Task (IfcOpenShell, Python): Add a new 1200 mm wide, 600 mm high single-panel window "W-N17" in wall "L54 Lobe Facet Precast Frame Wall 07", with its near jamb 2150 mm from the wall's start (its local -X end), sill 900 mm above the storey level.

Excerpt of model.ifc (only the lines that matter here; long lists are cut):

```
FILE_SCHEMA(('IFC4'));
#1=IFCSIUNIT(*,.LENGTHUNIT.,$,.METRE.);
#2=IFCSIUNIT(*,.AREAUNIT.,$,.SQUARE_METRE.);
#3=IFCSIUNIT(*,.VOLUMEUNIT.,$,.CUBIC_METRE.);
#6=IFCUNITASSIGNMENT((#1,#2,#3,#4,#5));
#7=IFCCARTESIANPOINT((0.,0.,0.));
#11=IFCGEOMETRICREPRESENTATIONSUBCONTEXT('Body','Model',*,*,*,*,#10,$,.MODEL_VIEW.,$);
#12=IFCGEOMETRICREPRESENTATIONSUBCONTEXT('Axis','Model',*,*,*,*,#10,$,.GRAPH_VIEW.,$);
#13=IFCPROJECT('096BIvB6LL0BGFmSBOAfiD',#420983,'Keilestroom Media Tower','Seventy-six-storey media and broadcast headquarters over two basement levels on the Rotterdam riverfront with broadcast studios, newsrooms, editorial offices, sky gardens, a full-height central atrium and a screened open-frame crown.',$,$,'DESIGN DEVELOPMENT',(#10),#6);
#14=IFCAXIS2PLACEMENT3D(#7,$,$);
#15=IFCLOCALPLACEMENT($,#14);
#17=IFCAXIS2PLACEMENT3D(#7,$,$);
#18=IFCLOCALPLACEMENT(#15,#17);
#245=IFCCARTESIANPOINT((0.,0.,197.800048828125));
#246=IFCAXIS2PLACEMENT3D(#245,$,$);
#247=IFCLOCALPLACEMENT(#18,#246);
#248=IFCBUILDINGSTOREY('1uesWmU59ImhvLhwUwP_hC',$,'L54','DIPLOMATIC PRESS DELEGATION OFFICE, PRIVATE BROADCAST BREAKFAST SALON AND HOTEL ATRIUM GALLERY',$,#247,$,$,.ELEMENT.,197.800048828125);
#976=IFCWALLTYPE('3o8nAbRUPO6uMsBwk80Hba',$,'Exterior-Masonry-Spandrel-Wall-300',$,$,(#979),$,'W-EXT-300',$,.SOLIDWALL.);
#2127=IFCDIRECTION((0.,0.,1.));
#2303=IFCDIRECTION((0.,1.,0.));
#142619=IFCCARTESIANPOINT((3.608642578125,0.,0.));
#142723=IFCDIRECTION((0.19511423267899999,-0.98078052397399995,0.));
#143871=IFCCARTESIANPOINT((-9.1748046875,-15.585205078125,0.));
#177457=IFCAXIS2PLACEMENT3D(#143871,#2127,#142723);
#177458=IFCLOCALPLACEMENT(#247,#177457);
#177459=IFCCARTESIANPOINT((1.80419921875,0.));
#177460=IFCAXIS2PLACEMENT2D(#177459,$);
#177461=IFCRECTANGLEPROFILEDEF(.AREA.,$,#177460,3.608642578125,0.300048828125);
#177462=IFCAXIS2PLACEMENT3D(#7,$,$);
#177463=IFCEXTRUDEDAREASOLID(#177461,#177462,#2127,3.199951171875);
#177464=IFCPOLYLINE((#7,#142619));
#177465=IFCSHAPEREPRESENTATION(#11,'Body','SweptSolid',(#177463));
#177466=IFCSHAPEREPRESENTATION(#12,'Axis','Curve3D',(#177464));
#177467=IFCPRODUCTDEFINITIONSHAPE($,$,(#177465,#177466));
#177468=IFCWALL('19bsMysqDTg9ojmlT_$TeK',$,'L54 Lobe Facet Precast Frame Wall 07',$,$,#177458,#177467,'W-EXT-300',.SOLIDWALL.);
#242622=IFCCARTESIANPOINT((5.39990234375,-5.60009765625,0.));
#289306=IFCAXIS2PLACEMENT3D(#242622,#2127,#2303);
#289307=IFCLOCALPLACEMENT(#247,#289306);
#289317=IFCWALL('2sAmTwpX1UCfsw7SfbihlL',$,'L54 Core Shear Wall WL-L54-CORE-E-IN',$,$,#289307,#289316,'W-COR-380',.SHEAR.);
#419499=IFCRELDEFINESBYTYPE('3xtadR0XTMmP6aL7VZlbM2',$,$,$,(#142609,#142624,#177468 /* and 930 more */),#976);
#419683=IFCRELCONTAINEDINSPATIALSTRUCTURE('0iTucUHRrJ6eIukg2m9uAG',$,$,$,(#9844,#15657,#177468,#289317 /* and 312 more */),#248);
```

```python
import numpy as np
import ifcopenshell
import ifcopenshell.api.feature
import ifcopenshell.api.geometry
import ifcopenshell.api.root
import ifcopenshell.api.spatial
import ifcopenshell.geom
import ifcopenshell.util.element
import ifcopenshell.util.placement
import ifcopenshell.util.representation
import ifcopenshell.util.shape
import ifcopenshell.util.unit

model = ifcopenshell.open("model.ifc")
unit_scale = ifcopenshell.util.unit.calculate_unit_scale(model)
settings = ifcopenshell.geom.settings()


def volume(element):
    """Net volume in cubic metres, openings subtracted."""
    shape = ifcopenshell.geom.create_shape(settings, element)
    return ifcopenshell.util.shape.get_volume(shape.geometry)


wall = model.by_guid("19bsMysqDTg9ojmlT_$TeK")
storey = ifcopenshell.util.element.get_container(wall, ifc_class="IfcBuildingStorey")
context = ifcopenshell.util.representation.get_context(model, "Model", "Body", "MODEL_VIEW")
before = volume(wall)

width, height, from_end, sill = 1.2, 0.6, 2.15, 0.9  # metres

# The wall runs along its own X axis, and the end named is its -X end.
wall_shape = ifcopenshell.geom.create_shape(settings, wall)
x, y, z = ifcopenshell.util.shape.get_vertices(wall_shape.geometry).T
start = x.min() + from_end
face, thickness = float(y.min()), float(y.max() - y.min())
wall_matrix = ifcopenshell.util.placement.get_local_placement(wall.ObjectPlacement)
level = ifcopenshell.util.placement.get_local_placement(storey.ObjectPlacement)[2, 3]


def in_wall(x, y):
    """Placement at x, y metres in the wall's axes, at sill height."""
    matrix = wall_matrix.copy()
    matrix[:, 3] = wall_matrix @ np.array([x / unit_scale, y / unit_scale, 0.0, 1.0])
    matrix[2, 3] = level + sill / unit_scale
    return matrix


# Opening: a box that overshoots both wall faces by 50 mm.
opening = ifcopenshell.api.root.create_entity(model, ifc_class="IfcOpeningElement", predefined_type="OPENING")
box = ifcopenshell.api.geometry.add_wall_representation(
    model, context=context, length=width, height=height, thickness=thickness + 0.1
)
ifcopenshell.api.geometry.assign_representation(model, product=opening, representation=box)
ifcopenshell.api.geometry.edit_object_placement(model, product=opening, matrix=in_wall(start, face - 0.05), is_si=False)
ifcopenshell.api.feature.add_feature(model, feature=opening, element=wall)

window = ifcopenshell.api.root.create_entity(model, ifc_class="IfcWindow", name="W-N17", predefined_type="WINDOW")
window.OverallWidth, window.OverallHeight = width / unit_scale, height / unit_scale
window.PartitioningType = "SINGLE_PANEL"
body = ifcopenshell.api.geometry.add_window_representation(
    model,
    context=context,
    overall_width=window.OverallWidth,
    overall_height=window.OverallHeight,
    partition_type="SINGLE_PANEL",
)
ifcopenshell.api.geometry.assign_representation(model, product=window, representation=body)
ifcopenshell.api.spatial.assign_container(model, products=[window], relating_structure=storey)
ifcopenshell.api.feature.add_filling(model, opening=opening, element=window)

# Centre the window in the wall's thickness.
ifcopenshell.api.geometry.edit_object_placement(model, product=window, matrix=in_wall(start, face), is_si=False)
window_shape = ifcopenshell.geom.create_shape(settings, window)
depth = ifcopenshell.util.shape.get_vertices(window_shape.geometry)[:, 1]
offset = face + thickness / 2 - (depth.min() + depth.max()) / 2
ifcopenshell.api.geometry.edit_object_placement(model, product=window, matrix=in_wall(start, offset), is_si=False)

after = volume(wall)

print(f"wall volume {before:.3f} -> {after:.3f} m3")

model.write("model_rev.ifc")
```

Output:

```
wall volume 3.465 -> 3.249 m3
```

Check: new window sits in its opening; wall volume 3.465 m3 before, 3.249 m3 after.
